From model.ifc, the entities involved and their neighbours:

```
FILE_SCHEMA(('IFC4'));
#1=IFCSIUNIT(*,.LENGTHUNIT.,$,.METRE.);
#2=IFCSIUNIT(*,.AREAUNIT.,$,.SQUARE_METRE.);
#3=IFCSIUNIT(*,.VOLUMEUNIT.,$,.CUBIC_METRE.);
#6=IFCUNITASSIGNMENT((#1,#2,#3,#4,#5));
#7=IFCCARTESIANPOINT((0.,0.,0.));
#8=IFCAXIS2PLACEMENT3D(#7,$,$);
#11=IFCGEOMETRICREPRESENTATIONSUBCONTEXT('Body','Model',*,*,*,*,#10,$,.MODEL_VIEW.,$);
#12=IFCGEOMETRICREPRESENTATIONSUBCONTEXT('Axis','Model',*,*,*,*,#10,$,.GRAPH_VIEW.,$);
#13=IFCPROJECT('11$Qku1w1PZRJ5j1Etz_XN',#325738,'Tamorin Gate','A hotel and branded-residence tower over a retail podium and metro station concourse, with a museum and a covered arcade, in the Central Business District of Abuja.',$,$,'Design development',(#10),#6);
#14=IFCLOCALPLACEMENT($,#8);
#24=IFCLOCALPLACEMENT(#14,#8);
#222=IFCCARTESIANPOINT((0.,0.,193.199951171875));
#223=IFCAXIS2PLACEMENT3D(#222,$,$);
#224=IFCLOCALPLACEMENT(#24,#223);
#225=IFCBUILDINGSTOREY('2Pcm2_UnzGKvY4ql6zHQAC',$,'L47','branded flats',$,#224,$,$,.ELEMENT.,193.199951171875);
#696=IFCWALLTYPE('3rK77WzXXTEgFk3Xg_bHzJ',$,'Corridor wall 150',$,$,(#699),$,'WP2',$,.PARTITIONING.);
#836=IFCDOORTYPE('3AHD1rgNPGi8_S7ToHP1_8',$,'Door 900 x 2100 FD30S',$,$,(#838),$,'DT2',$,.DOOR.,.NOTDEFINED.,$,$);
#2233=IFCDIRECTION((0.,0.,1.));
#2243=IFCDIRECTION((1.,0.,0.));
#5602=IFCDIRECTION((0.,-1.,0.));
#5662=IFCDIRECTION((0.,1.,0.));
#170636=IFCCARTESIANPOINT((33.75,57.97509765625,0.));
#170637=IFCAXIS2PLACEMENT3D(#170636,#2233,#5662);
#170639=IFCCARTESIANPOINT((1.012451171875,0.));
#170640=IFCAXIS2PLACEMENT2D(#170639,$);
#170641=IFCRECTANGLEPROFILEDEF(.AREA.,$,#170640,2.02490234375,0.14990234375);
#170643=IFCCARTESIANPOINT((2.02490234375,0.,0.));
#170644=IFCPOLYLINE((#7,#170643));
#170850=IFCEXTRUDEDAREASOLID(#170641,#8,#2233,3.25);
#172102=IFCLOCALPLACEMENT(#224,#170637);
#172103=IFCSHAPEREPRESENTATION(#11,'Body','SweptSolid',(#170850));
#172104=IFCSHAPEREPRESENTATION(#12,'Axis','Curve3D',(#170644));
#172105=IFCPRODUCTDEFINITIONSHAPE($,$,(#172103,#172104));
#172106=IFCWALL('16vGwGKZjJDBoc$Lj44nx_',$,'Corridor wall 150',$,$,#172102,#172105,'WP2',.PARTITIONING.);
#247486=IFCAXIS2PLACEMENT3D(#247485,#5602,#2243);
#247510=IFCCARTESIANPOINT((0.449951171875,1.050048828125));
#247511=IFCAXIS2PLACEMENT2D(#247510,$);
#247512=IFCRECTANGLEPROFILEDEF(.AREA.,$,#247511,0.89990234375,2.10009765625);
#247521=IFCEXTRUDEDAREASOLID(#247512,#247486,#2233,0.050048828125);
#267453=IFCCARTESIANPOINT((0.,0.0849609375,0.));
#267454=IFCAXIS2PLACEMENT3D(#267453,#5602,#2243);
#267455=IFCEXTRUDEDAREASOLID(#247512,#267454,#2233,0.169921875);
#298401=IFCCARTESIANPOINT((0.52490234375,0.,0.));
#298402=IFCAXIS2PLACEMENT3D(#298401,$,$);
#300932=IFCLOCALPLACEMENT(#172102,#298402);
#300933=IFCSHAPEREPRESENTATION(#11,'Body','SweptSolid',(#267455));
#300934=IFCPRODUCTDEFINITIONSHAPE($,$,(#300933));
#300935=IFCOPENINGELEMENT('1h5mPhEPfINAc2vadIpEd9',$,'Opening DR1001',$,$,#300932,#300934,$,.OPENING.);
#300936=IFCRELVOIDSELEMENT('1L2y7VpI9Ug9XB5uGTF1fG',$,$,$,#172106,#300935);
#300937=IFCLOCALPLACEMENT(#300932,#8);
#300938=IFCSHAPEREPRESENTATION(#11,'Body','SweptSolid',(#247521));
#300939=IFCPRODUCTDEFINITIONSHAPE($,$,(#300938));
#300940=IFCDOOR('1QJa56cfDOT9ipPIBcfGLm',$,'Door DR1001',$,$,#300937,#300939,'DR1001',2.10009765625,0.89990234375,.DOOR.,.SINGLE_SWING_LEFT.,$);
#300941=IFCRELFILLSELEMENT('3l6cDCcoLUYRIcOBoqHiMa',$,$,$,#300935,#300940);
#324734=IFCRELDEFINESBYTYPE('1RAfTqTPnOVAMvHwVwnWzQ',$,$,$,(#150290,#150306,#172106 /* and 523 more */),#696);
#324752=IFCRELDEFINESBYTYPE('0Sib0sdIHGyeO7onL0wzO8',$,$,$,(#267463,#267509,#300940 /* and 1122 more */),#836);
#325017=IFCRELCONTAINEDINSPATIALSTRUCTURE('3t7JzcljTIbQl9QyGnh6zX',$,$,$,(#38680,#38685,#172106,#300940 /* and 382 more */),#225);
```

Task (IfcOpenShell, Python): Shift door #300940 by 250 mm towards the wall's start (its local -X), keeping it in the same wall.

```python
import ifcopenshell
import ifcopenshell.api.geometry
import ifcopenshell.util.placement
import ifcopenshell.util.unit

model = ifcopenshell.open("model.ifc")
unit_scale = ifcopenshell.util.unit.calculate_unit_scale(model)

door = model.by_id(300940)
opening = door.FillsVoids[0].RelatingOpeningElement
wall = opening.VoidsElements[0].RelatingBuildingElement

wall_matrix = ifcopenshell.util.placement.get_local_placement(wall.ObjectPlacement)
shift = wall_matrix[:3, 0] * -0.25 / unit_scale
before = ifcopenshell.util.placement.get_local_placement(door.ObjectPlacement)[:3, 3].copy()

# The door is placed relative to its opening, so it follows when the opening moves.
matrix = ifcopenshell.util.placement.get_local_placement(opening.ObjectPlacement)
matrix[:3, 3] += shift
ifcopenshell.api.geometry.edit_object_placement(
    model, product=opening, matrix=matrix, is_si=False, should_transform_children=True
)

after = ifcopenshell.util.placement.get_local_placement(door.ObjectPlacement)[:3, 3]
print("door moved by", (after - before).round(3) + 0.0)

model.write("model_edited.ifc")
```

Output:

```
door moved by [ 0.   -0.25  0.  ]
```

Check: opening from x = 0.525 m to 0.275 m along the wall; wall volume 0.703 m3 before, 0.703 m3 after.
